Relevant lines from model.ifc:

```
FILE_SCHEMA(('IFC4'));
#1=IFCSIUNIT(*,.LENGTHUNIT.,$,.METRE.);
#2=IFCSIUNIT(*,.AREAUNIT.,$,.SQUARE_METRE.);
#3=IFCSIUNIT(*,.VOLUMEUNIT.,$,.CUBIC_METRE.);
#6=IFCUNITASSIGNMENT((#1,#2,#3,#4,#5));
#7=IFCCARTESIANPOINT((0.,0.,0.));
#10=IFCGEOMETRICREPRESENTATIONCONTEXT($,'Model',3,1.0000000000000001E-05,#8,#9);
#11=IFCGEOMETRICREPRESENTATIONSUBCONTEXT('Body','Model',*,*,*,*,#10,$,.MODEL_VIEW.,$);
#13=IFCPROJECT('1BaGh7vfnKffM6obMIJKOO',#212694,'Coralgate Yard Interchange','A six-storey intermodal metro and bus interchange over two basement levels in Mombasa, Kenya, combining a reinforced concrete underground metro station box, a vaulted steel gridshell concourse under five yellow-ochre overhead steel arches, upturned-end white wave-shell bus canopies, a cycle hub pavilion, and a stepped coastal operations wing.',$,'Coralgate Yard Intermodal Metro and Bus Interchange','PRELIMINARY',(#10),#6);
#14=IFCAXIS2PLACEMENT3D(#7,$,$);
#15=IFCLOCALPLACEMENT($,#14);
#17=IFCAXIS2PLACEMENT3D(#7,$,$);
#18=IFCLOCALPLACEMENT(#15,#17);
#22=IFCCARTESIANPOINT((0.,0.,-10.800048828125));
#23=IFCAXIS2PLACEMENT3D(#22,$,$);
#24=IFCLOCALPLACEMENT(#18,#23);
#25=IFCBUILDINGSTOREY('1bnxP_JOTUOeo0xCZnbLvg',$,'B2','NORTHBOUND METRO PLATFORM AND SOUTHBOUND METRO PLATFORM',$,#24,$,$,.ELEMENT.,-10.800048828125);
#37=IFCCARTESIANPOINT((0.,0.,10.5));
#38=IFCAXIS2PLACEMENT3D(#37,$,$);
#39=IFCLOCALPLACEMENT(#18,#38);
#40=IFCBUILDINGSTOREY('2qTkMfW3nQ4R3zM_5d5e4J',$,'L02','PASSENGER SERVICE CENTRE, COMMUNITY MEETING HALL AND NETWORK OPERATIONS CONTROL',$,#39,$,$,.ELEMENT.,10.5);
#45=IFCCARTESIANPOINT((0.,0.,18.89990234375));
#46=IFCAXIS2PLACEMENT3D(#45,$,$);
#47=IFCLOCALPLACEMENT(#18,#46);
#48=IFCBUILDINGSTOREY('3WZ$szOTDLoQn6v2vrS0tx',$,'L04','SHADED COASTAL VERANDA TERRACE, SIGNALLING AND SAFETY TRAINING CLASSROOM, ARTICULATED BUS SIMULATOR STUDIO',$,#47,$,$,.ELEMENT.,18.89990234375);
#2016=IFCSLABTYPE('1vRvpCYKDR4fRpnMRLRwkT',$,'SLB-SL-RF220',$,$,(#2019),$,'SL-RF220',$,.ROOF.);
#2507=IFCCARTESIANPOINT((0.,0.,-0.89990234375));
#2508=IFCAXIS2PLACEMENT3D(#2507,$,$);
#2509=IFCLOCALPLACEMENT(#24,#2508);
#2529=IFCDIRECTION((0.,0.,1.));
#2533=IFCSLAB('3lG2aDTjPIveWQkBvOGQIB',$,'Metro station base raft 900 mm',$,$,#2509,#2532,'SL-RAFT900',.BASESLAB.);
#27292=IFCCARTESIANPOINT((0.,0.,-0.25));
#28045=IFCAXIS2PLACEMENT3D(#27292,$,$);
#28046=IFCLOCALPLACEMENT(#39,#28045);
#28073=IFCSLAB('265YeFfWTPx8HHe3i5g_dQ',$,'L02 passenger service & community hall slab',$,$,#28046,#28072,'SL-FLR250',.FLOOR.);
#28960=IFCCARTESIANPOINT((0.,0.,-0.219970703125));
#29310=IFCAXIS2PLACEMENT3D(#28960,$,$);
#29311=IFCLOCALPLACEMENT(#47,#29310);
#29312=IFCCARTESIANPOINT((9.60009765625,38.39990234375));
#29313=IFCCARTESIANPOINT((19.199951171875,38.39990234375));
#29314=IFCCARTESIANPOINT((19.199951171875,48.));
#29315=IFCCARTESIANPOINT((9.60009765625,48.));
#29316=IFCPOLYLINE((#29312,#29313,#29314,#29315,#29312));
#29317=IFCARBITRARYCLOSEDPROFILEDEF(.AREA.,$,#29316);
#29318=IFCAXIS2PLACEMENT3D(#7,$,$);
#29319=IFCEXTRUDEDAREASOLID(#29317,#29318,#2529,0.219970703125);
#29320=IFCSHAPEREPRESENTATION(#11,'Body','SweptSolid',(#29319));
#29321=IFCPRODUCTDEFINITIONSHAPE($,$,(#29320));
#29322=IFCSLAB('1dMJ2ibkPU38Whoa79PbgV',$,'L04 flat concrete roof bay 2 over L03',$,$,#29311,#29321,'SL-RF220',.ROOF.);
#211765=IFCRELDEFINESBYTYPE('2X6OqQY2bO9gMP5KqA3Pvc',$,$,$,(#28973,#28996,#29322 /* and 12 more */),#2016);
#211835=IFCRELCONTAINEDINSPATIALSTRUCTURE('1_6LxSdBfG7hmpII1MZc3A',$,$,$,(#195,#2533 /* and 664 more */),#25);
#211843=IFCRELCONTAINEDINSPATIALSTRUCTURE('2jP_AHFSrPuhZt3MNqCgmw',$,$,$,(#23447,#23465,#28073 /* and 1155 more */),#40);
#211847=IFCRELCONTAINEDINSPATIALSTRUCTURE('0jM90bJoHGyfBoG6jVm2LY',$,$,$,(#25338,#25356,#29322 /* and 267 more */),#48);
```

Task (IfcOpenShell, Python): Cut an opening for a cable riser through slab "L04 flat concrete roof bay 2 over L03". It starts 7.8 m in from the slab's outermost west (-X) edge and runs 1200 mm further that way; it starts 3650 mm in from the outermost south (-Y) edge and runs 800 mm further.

```python
import numpy as np
import ifcopenshell
import ifcopenshell.api.feature
import ifcopenshell.api.geometry
import ifcopenshell.api.root
import ifcopenshell.geom
import ifcopenshell.util.placement
import ifcopenshell.util.representation
import ifcopenshell.util.shape
import ifcopenshell.util.unit

model = ifcopenshell.open("model.ifc")
unit_scale = ifcopenshell.util.unit.calculate_unit_scale(model)
settings = ifcopenshell.geom.settings()


def volume(element):
    """Net volume in cubic metres, openings subtracted."""
    shape = ifcopenshell.geom.create_shape(settings, element)
    return ifcopenshell.util.shape.get_volume(shape.geometry)


slab = model.by_guid("1dMJ2ibkPU38Whoa79PbgV")
before = volume(slab)

# Extent in the slab's own axes, in metres. The edges named are its -X and -Y sides.
slab_shape = ifcopenshell.geom.create_shape(settings, slab)
vertices = ifcopenshell.util.shape.get_vertices(slab_shape.geometry)
x_min, y_min, bottom = vertices.min(axis=0)
top = vertices[:, 2].max()

opening = ifcopenshell.api.root.create_entity(model, ifc_class="IfcOpeningElement", name="Cable riser opening", predefined_type="OPENING")
context = ifcopenshell.util.representation.get_context(model, "Model", "Body", "MODEL_VIEW")
width, depth = 1.2, 0.8
outline = [(0.0, 0.0), (width, 0.0), (width, depth), (0.0, depth), (0.0, 0.0)]
# Overshoot both faces by 50 mm so the cut is clean.
shape = ifcopenshell.api.geometry.add_slab_representation(
    model, context=context, depth=top - bottom + 0.1, polyline=outline
)
ifcopenshell.api.geometry.assign_representation(model, product=opening, representation=shape)

matrix = ifcopenshell.util.placement.get_local_placement(slab.ObjectPlacement)
matrix[:, 3] = matrix @ np.append(np.array([x_min + 7.8, y_min + 3.65, bottom - 0.05]) / unit_scale, 1.0)
ifcopenshell.api.geometry.edit_object_placement(model, product=opening, matrix=matrix, is_si=False)
ifcopenshell.api.feature.add_feature(model, feature=opening, element=slab)

after = volume(slab)

print(f"slab volume {before:.3f} -> {after:.3f} m3")

model.write("model-out.ifc")
```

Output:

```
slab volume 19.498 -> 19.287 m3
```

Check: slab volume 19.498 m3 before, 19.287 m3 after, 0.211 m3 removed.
